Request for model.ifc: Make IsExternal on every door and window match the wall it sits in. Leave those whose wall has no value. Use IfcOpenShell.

First a look at what the model holds.

```python
import ifcopenshell
import ifcopenshell.util.element

model = ifcopenshell.open("model.ifc")
print(model.schema)
seen = {}
for e in model.by_type("IfcDoor") + model.by_type("IfcWindow"):
    if not e.FillsVoids:
        continue
    host = e.FillsVoids[0].RelatingOpeningElement.VoidsElements[0].RelatingBuildingElement
    own = ifcopenshell.util.element.get_pset(e, f"Pset_{e.is_a()[3:].removesuffix('StandardCase')}Common", "IsExternal")
    wall = ifcopenshell.util.element.get_pset(host, "Pset_WallCommon", "IsExternal")
    seen[e.is_a(), own, wall] = seen.get((e.is_a(), own, wall), 0) + 1
for (cls, own, wall), count in sorted(seen.items(), key=str):
    print(count, cls, "IsExternal:", own, "| host wall:", wall)
```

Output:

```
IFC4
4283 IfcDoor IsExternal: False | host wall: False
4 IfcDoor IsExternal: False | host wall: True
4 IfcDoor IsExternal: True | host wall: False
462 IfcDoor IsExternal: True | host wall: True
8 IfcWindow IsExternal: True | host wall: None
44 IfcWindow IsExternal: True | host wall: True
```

```python
import ifcopenshell
import ifcopenshell.api.pset
import ifcopenshell.util.element

model = ifcopenshell.open("model.ifc")

count = 0
for ifc_class, pset_name in (("IfcDoor", "Pset_DoorCommon"), ("IfcWindow", "Pset_WindowCommon")):
    for e in model.by_type(ifc_class):
        if not e.FillsVoids:
            continue
        host = e.FillsVoids[0].RelatingOpeningElement.VoidsElements[0].RelatingBuildingElement
        external = ifcopenshell.util.element.get_pset(host, "Pset_WallCommon", "IsExternal")
        if external is None or ifcopenshell.util.element.get_pset(e, pset_name, "IsExternal") == external:
            continue
        pset = ifcopenshell.api.pset.add_pset(model, product=e, name=pset_name)
        ifcopenshell.api.pset.edit_pset(model, pset=pset, properties={"IsExternal": external})
        count += 1

print(count, "updated")

model.write("model_rev.ifc")
```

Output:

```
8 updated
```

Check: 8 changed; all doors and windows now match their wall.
